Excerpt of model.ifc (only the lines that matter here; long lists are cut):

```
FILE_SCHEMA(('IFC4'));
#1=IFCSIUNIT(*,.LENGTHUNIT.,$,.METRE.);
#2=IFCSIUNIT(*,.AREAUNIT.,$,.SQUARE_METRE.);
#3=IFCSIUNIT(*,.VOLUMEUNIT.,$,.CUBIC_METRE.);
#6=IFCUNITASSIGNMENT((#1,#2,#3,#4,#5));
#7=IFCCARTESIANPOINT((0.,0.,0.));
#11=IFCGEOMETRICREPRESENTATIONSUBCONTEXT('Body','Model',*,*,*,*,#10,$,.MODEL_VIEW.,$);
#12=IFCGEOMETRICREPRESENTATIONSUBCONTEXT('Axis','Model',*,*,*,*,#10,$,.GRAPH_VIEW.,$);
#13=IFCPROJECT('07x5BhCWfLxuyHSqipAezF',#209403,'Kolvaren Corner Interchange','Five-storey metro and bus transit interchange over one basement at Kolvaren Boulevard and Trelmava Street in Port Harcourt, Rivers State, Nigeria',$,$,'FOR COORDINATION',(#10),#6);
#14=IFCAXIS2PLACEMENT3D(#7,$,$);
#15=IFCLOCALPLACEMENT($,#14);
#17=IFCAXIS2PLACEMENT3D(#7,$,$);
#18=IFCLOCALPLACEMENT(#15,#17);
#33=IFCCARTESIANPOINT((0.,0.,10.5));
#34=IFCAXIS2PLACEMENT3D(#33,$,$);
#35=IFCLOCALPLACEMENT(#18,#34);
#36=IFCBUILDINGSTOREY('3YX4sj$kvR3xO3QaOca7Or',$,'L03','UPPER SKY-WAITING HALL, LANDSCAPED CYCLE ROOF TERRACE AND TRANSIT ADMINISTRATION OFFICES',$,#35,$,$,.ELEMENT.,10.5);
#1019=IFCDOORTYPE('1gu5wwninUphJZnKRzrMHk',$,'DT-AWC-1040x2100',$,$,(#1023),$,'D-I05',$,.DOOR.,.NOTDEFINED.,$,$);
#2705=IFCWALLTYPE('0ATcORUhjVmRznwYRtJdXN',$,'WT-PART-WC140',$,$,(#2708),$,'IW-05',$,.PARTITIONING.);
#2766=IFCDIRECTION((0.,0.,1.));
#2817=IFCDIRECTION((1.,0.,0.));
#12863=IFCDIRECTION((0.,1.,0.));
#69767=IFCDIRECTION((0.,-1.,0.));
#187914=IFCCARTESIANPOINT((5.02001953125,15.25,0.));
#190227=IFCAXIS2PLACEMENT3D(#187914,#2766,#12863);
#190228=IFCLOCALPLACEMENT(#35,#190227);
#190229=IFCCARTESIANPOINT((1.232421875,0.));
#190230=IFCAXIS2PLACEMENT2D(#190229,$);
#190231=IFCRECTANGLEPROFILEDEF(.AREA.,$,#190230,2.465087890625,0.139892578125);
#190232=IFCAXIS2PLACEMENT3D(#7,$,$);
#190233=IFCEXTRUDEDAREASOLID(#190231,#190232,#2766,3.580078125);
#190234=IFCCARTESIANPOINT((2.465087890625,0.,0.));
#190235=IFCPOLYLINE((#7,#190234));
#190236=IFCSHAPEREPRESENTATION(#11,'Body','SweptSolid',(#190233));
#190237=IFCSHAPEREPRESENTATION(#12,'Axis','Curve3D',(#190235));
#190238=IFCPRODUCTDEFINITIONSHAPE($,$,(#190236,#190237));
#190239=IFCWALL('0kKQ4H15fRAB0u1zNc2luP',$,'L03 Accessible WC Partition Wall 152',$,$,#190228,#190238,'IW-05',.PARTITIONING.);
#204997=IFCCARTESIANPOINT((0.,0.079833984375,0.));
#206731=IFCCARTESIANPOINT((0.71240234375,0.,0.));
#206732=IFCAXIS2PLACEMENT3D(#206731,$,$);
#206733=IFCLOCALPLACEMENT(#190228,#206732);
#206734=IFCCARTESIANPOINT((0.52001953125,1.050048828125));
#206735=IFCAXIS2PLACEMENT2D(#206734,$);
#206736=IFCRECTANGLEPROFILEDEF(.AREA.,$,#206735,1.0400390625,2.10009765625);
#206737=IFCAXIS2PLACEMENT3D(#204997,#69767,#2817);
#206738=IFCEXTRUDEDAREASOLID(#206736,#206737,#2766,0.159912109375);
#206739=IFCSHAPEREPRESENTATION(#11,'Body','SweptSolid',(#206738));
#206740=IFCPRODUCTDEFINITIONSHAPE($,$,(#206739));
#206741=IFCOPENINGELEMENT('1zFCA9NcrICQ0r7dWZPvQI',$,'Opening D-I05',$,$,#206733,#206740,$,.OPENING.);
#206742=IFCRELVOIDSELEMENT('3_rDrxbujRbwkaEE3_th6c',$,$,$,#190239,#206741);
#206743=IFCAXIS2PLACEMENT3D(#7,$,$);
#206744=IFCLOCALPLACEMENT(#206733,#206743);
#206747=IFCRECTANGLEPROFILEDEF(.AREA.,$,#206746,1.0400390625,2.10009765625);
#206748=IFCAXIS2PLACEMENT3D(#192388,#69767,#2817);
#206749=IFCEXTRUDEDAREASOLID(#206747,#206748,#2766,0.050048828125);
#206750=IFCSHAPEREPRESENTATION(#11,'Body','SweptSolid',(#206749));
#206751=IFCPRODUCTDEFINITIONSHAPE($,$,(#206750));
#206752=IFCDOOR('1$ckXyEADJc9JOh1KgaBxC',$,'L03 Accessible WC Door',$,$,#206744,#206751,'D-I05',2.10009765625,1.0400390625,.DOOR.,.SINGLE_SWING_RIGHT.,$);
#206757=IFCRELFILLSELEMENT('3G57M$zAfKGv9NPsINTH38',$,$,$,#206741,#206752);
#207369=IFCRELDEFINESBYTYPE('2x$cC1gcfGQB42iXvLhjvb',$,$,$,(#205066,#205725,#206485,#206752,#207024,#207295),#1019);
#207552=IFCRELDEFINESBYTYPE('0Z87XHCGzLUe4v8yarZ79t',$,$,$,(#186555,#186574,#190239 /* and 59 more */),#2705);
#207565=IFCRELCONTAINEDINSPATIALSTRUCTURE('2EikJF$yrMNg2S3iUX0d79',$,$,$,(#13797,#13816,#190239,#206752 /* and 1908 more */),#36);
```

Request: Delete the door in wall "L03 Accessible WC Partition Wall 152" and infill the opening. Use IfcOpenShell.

```python
import ifcopenshell
import ifcopenshell.api.feature
import ifcopenshell.api.root
import ifcopenshell.geom
import ifcopenshell.util.shape

model = ifcopenshell.open("model.ifc")
settings = ifcopenshell.geom.settings()


def volume(element):
    """Net volume in cubic metres, openings subtracted."""
    shape = ifcopenshell.geom.create_shape(settings, element)
    return ifcopenshell.util.shape.get_volume(shape.geometry)


door = model.by_guid("1$ckXyEADJc9JOh1KgaBxC")
opening = door.FillsVoids[0].RelatingOpeningElement
wall = opening.VoidsElements[0].RelatingBuildingElement
before = volume(wall)

ifcopenshell.api.root.remove_product(model, product=door)
ifcopenshell.api.feature.remove_feature(model, feature=opening)

after = volume(wall)

print(f"wall volume {before:.3f} -> {after:.3f} m3")

model.write("model_updated.ifc")
```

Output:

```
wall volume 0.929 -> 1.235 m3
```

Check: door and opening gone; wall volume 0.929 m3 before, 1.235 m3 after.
